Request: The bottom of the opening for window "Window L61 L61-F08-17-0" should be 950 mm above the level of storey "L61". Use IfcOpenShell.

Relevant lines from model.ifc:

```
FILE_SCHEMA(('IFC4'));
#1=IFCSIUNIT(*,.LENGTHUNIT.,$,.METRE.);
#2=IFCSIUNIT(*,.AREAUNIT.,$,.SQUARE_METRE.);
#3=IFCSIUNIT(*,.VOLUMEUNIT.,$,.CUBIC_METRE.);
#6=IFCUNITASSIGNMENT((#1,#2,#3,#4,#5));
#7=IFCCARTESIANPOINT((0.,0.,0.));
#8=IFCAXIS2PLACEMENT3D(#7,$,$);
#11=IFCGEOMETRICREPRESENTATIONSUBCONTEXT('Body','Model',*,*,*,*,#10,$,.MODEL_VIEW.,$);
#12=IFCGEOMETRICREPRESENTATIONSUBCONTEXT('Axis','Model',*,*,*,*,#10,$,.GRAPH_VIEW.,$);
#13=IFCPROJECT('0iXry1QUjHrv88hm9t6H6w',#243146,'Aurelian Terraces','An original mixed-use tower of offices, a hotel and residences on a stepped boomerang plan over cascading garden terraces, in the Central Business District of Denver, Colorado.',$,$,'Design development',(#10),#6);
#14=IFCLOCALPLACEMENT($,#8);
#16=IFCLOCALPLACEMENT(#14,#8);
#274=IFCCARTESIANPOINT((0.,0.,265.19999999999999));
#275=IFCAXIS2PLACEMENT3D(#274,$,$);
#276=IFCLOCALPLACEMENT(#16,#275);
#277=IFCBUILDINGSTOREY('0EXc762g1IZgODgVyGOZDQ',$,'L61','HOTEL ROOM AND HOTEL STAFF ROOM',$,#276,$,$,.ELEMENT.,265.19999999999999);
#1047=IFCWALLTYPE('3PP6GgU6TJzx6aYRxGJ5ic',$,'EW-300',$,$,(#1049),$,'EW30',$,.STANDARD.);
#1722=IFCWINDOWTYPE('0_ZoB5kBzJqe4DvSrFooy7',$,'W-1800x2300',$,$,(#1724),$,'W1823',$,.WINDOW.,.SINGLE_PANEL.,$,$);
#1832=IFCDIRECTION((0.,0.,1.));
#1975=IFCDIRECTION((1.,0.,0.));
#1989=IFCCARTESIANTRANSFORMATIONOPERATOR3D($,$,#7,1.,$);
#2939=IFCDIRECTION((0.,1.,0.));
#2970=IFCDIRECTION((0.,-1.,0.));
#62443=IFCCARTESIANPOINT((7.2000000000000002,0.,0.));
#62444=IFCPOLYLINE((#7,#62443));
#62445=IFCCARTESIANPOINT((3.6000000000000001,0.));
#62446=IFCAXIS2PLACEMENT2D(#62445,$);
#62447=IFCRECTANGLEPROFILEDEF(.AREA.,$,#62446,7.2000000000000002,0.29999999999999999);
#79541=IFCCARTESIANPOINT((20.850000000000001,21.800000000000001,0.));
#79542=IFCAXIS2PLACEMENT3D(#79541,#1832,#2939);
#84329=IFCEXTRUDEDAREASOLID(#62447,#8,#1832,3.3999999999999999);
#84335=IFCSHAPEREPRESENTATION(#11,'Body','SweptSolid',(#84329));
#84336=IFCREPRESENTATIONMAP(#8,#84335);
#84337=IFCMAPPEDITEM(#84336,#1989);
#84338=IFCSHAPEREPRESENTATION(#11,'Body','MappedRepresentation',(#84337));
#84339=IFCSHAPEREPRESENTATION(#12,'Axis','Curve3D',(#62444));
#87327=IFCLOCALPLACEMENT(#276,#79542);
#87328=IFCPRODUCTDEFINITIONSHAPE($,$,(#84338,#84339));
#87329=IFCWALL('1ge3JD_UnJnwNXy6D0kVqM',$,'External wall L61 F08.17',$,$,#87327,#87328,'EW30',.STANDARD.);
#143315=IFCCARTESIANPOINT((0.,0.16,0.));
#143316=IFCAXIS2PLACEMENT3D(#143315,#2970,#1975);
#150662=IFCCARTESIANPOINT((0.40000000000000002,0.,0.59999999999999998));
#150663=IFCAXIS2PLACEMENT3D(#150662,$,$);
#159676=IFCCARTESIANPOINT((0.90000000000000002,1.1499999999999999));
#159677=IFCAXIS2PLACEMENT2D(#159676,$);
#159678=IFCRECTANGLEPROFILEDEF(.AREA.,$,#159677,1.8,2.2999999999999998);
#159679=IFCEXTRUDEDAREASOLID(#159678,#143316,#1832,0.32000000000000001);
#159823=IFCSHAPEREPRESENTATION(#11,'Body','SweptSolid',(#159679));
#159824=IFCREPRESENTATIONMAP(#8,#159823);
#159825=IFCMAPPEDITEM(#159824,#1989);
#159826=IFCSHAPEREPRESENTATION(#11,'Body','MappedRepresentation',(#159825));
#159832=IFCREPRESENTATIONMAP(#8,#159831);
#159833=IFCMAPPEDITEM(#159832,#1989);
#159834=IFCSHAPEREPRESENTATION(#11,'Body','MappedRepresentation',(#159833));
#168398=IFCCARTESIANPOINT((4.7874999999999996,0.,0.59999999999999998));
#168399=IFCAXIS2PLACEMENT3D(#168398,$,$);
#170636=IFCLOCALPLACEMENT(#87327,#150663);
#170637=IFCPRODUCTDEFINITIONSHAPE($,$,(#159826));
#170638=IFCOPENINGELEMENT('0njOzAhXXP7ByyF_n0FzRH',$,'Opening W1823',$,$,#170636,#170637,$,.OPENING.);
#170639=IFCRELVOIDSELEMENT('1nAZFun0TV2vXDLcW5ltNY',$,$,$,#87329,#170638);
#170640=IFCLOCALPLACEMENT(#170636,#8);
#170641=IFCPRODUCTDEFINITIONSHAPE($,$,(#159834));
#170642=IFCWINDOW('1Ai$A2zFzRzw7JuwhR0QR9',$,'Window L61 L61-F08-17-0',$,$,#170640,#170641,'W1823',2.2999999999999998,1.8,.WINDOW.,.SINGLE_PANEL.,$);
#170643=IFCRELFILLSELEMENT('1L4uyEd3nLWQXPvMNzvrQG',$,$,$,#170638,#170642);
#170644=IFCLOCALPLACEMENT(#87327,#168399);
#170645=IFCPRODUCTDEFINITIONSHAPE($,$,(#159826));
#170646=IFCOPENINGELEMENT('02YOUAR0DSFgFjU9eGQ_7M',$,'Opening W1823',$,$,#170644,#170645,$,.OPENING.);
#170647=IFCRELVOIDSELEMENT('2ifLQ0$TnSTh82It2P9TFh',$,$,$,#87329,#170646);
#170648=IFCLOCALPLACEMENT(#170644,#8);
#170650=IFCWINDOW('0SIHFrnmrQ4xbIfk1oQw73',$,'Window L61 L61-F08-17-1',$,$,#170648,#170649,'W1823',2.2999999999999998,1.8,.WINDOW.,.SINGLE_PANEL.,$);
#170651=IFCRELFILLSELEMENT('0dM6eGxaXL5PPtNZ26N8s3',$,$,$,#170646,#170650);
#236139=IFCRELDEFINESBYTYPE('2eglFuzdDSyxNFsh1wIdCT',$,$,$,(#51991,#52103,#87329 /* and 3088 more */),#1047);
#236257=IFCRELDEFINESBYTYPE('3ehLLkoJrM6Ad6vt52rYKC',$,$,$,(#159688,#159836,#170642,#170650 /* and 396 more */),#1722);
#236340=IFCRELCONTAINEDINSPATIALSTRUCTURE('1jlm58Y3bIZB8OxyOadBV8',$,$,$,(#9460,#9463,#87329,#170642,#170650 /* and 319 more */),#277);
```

```python
import numpy as np
import ifcopenshell
import ifcopenshell.api.geometry
import ifcopenshell.geom
import ifcopenshell.util.element
import ifcopenshell.util.placement
import ifcopenshell.util.shape
import ifcopenshell.util.unit

model = ifcopenshell.open("model.ifc")
unit_scale = ifcopenshell.util.unit.calculate_unit_scale(model)

window = model.by_guid("1Ai$A2zFzRzw7JuwhR0QR9")
opening = window.FillsVoids[0].RelatingOpeningElement
storey = ifcopenshell.util.element.get_container(window, ifc_class="IfcBuildingStorey")
level = ifcopenshell.util.placement.get_local_placement(storey.ObjectPlacement)[2, 3]

# The opening's origin need not be at the sill, so measure its lowest point.
shape = ifcopenshell.geom.create_shape(ifcopenshell.geom.settings(), opening)
bottom = ifcopenshell.util.shape.get_shape_bottom_elevation(shape, shape.geometry) / unit_scale
dz = level + 0.95 / unit_scale - bottom

shift = np.array([0.0, 0.0, dz])
# The window is placed relative to its opening, so it follows when the opening moves.
matrix = ifcopenshell.util.placement.get_local_placement(opening.ObjectPlacement)
matrix[:3, 3] += shift
ifcopenshell.api.geometry.edit_object_placement(
    model, product=opening, matrix=matrix, is_si=False, should_transform_children=True
)

print(f"moved by {dz * unit_scale:+.3f} m")

model.write("model-out.ifc")
```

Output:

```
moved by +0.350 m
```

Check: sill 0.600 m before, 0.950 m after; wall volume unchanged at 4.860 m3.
